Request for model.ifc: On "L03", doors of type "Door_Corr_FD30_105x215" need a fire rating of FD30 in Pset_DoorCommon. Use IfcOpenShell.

First a look at what the model holds.

```python
import ifcopenshell
import ifcopenshell.util.element

model = ifcopenshell.open("model.ifc")
print(model.schema)
storey = next(s for s in model.by_type("IfcBuildingStorey") if s.Name == "L03")
doors = [e for e in ifcopenshell.util.element.get_decomposition(storey) if e.is_a("IfcDoor")]
seen = {}
for e in doors:
    element_type = ifcopenshell.util.element.get_type(e)
    key = (element_type.Name if element_type != e and element_type else None, ifcopenshell.util.element.get_pset(e, "Pset_DoorCommon", "FireRating"))
    seen[key] = seen.get(key, 0) + 1
for (name, value), count in sorted(seen.items(), key=str):
    print(count, "x", name, "|", value)
```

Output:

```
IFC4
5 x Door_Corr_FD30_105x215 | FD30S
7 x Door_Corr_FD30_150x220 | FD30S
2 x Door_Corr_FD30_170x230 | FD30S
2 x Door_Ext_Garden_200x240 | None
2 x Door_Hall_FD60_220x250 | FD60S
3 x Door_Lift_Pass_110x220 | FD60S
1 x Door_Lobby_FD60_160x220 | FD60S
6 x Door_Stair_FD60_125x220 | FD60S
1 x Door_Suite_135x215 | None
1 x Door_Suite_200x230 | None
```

```python
import ifcopenshell
import ifcopenshell.api.pset
import ifcopenshell.util.element

model = ifcopenshell.open("model.ifc")

storey = next(s for s in model.by_type("IfcBuildingStorey") if s.Name == "L03")
doors = [e for e in ifcopenshell.util.element.get_decomposition(storey) if e.is_a("IfcDoor")]

count = 0
for e in doors:
    element_type = ifcopenshell.util.element.get_type(e)
    if element_type in (None, e) or element_type.Name != "Door_Corr_FD30_105x215":
        continue
    # add_pset returns the element's existing set when there is one.
    pset = ifcopenshell.api.pset.add_pset(model, product=e, name="Pset_DoorCommon")
    ifcopenshell.api.pset.edit_pset(model, pset=pset, properties={"FireRating": "FD30"})
    count += 1

print(count, "doors updated")

model.write("model_edited.ifc")
```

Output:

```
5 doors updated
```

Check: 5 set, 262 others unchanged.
